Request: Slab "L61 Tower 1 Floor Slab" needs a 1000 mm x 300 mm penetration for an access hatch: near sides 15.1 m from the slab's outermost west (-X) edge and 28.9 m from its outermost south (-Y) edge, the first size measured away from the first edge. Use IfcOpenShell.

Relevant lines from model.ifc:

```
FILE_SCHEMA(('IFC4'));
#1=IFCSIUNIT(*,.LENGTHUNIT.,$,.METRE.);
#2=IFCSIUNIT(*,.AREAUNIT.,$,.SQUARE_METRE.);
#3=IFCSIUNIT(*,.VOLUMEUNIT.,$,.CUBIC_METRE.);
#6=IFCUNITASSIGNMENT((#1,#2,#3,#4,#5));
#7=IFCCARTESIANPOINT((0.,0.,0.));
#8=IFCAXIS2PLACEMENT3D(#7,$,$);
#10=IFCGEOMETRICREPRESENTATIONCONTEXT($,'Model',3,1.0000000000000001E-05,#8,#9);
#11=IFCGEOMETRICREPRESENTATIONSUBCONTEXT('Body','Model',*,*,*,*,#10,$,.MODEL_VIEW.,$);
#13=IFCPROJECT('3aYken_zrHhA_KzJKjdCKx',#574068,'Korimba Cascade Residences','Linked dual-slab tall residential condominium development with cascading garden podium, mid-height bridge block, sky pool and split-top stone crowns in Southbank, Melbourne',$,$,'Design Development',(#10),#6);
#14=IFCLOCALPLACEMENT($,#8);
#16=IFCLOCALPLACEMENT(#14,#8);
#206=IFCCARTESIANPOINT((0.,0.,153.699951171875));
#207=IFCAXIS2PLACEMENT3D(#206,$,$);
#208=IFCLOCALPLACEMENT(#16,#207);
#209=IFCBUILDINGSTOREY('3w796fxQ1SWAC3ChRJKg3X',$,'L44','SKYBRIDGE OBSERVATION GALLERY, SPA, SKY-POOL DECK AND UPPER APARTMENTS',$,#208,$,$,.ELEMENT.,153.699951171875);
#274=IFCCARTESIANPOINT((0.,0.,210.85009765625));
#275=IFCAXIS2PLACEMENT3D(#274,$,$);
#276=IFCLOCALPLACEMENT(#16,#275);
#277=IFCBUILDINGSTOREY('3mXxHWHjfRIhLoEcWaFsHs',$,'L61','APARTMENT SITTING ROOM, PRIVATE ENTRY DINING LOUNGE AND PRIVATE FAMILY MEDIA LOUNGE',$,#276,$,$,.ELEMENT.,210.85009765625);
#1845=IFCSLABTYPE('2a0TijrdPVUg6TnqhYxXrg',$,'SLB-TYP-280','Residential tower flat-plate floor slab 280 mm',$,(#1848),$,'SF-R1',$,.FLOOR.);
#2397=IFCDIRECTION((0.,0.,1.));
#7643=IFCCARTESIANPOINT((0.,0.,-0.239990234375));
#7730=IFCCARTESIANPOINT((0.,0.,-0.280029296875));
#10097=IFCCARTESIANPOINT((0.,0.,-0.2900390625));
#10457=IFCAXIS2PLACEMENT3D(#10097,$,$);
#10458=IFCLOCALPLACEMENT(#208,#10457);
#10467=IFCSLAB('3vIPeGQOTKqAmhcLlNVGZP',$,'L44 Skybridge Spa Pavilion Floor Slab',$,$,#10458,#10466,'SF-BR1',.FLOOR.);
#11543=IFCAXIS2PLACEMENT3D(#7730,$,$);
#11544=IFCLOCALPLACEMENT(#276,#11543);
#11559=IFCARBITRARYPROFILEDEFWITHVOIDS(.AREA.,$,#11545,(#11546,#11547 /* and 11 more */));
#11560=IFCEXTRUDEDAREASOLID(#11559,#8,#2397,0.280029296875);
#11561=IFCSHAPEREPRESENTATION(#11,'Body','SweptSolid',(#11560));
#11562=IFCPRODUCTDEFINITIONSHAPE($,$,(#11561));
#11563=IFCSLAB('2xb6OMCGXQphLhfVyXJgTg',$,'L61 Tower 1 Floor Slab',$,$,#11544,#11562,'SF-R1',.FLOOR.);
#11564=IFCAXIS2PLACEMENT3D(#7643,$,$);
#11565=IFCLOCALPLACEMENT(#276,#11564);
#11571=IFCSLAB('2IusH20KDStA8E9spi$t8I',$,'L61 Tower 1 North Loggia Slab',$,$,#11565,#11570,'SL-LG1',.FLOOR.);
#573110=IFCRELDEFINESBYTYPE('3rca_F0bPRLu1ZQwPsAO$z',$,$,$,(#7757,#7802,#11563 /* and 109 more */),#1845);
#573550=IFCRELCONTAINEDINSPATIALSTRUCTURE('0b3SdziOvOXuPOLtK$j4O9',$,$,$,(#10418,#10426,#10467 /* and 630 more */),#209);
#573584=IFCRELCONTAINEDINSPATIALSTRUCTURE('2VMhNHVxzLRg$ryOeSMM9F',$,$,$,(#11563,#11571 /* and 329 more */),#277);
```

```python
import numpy as np
import ifcopenshell
import ifcopenshell.api.feature
import ifcopenshell.api.geometry
import ifcopenshell.api.root
import ifcopenshell.geom
import ifcopenshell.util.placement
import ifcopenshell.util.representation
import ifcopenshell.util.shape
import ifcopenshell.util.unit

model = ifcopenshell.open("model.ifc")
unit_scale = ifcopenshell.util.unit.calculate_unit_scale(model)
settings = ifcopenshell.geom.settings()


def volume(element):
    """Net volume in cubic metres, openings subtracted."""
    shape = ifcopenshell.geom.create_shape(settings, element)
    return ifcopenshell.util.shape.get_volume(shape.geometry)


slab = model.by_guid("2xb6OMCGXQphLhfVyXJgTg")
before = volume(slab)

# Extent in the slab's own axes, in metres. The edges named are its -X and -Y sides.
slab_shape = ifcopenshell.geom.create_shape(settings, slab)
vertices = ifcopenshell.util.shape.get_vertices(slab_shape.geometry)
x_min, y_min, bottom = vertices.min(axis=0)
top = vertices[:, 2].max()

opening = ifcopenshell.api.root.create_entity(model, ifc_class="IfcOpeningElement", name="Access hatch opening", predefined_type="OPENING")
context = ifcopenshell.util.representation.get_context(model, "Model", "Body", "MODEL_VIEW")
width, depth = 1, 0.3
outline = [(0.0, 0.0), (width, 0.0), (width, depth), (0.0, depth), (0.0, 0.0)]
# Overshoot both faces by 50 mm so the cut is clean.
shape = ifcopenshell.api.geometry.add_slab_representation(
    model, context=context, depth=top - bottom + 0.1, polyline=outline
)
ifcopenshell.api.geometry.assign_representation(model, product=opening, representation=shape)

matrix = ifcopenshell.util.placement.get_local_placement(slab.ObjectPlacement)
matrix[:, 3] = matrix @ np.append(np.array([x_min + 15.1, y_min + 28.9, bottom - 0.05]) / unit_scale, 1.0)
ifcopenshell.api.geometry.edit_object_placement(model, product=opening, matrix=matrix, is_si=False)
ifcopenshell.api.feature.add_feature(model, feature=opening, element=slab)

after = volume(slab)

print(f"slab volume {before:.3f} -> {after:.3f} m3")

model.write("model_v2.ifc")
```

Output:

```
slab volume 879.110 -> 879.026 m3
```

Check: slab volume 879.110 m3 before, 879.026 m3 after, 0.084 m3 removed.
